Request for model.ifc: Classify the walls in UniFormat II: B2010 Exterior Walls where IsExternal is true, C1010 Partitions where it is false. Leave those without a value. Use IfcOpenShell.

First a look at what the model holds.

```python
import ifcopenshell
import ifcopenshell.util.element

model = ifcopenshell.open("model.ifc")
print(model.schema)
print("classifications:", [c.Name for c in model.by_type("IfcClassification")])
values = [ifcopenshell.util.element.get_pset(e, "Pset_WallCommon", "IsExternal") for e in model.by_type("IfcWall")]
for value in (True, False, None):
    print("IsExternal", value, values.count(value))
```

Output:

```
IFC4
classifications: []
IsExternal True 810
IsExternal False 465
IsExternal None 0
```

```python
import ifcopenshell
import ifcopenshell.api.classification
import ifcopenshell.util.element

model = ifcopenshell.open("model.ifc")

system = ifcopenshell.api.classification.add_classification(model, classification="UniFormat II")

walls = model.by_type("IfcWall")
external = {e: ifcopenshell.util.element.get_pset(e, "Pset_WallCommon", "IsExternal") for e in walls}
for flag, code, name in ((True, "B2010", "Exterior Walls"), (False, "C1010", "Partitions")):
    products = [e for e in walls if external[e] is flag]
    ifcopenshell.api.classification.add_reference(
        model, products=products, classification=system, identification=code, name=name
    )
    print(code, len(products))

model.write("model_updated.ifc")
```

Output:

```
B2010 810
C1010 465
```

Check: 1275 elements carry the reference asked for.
